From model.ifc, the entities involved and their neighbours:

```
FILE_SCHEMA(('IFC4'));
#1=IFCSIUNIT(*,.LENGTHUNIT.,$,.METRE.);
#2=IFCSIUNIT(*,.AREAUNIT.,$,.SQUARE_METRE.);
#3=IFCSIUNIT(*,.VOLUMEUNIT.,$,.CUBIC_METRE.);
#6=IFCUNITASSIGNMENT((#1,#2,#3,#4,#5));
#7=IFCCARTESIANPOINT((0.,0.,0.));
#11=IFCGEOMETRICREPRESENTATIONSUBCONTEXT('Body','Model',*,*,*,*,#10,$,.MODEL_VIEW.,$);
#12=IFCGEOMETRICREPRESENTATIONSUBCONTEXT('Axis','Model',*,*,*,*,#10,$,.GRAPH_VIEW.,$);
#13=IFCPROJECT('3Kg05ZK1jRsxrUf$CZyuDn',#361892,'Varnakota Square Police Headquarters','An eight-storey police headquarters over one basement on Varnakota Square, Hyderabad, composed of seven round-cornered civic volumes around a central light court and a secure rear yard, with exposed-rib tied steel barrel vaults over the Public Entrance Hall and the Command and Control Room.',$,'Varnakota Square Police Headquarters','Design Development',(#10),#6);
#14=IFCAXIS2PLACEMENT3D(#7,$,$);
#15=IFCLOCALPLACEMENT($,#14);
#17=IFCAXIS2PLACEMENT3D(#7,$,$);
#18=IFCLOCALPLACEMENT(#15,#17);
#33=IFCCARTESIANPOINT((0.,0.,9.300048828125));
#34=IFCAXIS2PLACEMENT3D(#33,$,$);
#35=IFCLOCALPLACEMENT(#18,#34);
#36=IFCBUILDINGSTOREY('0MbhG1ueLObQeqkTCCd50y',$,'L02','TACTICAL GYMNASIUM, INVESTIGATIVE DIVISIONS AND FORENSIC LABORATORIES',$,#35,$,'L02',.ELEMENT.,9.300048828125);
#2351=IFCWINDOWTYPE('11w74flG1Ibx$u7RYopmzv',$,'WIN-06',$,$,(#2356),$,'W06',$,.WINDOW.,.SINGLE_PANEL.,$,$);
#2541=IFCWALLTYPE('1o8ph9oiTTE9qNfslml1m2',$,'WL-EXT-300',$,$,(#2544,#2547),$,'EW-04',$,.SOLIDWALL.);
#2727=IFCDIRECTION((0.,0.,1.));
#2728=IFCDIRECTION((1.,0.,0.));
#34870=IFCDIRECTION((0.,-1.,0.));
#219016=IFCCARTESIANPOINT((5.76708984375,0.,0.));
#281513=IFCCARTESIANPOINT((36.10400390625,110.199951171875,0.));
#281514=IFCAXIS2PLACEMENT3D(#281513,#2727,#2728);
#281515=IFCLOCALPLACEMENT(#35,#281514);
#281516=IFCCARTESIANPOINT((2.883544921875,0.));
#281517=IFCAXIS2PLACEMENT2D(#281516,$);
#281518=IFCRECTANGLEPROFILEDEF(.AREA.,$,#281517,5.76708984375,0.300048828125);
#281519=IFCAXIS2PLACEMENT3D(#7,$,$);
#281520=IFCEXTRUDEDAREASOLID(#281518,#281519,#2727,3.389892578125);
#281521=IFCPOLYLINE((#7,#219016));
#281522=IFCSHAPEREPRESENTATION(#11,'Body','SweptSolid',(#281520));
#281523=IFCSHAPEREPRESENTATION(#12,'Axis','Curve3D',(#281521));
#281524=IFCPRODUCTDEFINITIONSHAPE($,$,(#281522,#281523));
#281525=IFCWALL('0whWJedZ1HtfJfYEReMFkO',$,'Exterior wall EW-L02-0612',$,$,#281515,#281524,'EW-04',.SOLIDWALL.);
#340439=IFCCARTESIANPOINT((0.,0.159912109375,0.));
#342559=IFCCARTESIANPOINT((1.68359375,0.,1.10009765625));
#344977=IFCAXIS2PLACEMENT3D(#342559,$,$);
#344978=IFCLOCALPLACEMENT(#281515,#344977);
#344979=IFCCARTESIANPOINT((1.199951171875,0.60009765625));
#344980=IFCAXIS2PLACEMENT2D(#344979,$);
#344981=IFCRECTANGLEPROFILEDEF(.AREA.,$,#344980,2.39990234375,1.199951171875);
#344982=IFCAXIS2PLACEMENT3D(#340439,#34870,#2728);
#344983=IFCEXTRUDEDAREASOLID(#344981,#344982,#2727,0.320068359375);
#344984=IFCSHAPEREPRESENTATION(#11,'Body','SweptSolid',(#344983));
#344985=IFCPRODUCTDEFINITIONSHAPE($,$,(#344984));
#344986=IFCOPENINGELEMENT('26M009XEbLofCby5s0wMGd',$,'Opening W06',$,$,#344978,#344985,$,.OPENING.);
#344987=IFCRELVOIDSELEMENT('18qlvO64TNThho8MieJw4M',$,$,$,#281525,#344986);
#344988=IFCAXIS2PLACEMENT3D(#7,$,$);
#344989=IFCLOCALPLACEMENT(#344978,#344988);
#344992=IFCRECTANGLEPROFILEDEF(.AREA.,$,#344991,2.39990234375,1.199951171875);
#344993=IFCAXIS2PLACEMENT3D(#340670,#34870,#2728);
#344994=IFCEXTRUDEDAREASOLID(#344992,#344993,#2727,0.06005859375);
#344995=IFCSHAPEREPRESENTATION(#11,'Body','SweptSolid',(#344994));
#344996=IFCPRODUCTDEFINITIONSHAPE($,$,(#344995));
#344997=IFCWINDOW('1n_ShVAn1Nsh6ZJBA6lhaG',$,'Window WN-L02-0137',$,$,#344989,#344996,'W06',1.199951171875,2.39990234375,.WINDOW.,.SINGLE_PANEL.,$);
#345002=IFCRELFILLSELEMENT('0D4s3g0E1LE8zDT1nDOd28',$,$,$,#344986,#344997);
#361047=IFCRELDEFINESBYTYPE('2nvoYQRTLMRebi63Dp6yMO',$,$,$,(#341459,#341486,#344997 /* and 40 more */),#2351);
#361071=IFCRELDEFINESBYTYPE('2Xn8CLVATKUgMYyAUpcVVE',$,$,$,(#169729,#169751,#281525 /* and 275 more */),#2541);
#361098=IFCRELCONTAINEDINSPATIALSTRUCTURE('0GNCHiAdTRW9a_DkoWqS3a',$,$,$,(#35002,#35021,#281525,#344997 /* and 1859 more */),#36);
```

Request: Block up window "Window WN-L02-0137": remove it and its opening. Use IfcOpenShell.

```python
import ifcopenshell
import ifcopenshell.api.feature
import ifcopenshell.api.root
import ifcopenshell.geom
import ifcopenshell.util.shape

model = ifcopenshell.open("model.ifc")
settings = ifcopenshell.geom.settings()


def volume(element):
    """Net volume in cubic metres, openings subtracted."""
    shape = ifcopenshell.geom.create_shape(settings, element)
    return ifcopenshell.util.shape.get_volume(shape.geometry)


window = model.by_guid("1n_ShVAn1Nsh6ZJBA6lhaG")
opening = window.FillsVoids[0].RelatingOpeningElement
wall = opening.VoidsElements[0].RelatingBuildingElement
before = volume(wall)

ifcopenshell.api.root.remove_product(model, product=window)
ifcopenshell.api.feature.remove_feature(model, feature=opening)

after = volume(wall)

print(f"wall volume {before:.3f} -> {after:.3f} m3")

model.write("model_rev.ifc")
```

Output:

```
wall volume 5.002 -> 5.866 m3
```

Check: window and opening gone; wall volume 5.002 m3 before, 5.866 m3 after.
